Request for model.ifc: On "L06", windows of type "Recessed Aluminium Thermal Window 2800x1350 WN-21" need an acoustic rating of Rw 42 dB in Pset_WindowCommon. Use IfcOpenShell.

First a look at what the model holds.

```python
import ifcopenshell
import ifcopenshell.util.element

model = ifcopenshell.open("model.ifc")
print(model.schema)
storey = next(s for s in model.by_type("IfcBuildingStorey") if s.Name == "L06")
windows = [e for e in ifcopenshell.util.element.get_decomposition(storey) if e.is_a("IfcWindow")]
seen = {}
for e in windows:
    element_type = ifcopenshell.util.element.get_type(e)
    key = (element_type.Name if element_type != e and element_type else None, ifcopenshell.util.element.get_pset(e, "Pset_WindowCommon", "AcousticRating"))
    seen[key] = seen.get(key, 0) + 1
for (name, value), count in sorted(seen.items(), key=str):
    print(count, "x", name, "|", value)
```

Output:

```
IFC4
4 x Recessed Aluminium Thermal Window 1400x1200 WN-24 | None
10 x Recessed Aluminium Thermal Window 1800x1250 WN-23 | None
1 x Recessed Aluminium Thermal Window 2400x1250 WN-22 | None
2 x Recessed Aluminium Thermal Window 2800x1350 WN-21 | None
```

```python
import ifcopenshell
import ifcopenshell.api.pset
import ifcopenshell.util.element

model = ifcopenshell.open("model.ifc")

storey = next(s for s in model.by_type("IfcBuildingStorey") if s.Name == "L06")
windows = [e for e in ifcopenshell.util.element.get_decomposition(storey) if e.is_a("IfcWindow")]

count = 0
for e in windows:
    element_type = ifcopenshell.util.element.get_type(e)
    if element_type in (None, e) or element_type.Name != "Recessed Aluminium Thermal Window 2800x1350 WN-21":
        continue
    # add_pset returns the element's existing set when there is one.
    pset = ifcopenshell.api.pset.add_pset(model, product=e, name="Pset_WindowCommon")
    ifcopenshell.api.pset.edit_pset(model, pset=pset, properties={"AcousticRating": "Rw 42 dB"})
    count += 1

print(count, "windows updated")

model.write("model_edited.ifc")
```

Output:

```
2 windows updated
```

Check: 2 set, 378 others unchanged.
